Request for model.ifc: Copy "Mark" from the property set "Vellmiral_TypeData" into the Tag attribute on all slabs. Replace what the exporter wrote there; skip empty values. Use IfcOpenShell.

First a look at what the model holds.

```python
import ifcopenshell
import ifcopenshell.util.element

model = ifcopenshell.open("model.ifc")
print(model.schema)
slabs = model.by_type("IfcSlab")
print(len(slabs), "slabs")
for e in slabs[:8]:
    source = ifcopenshell.util.element.get_pset(e, "Vellmiral_TypeData", "Mark")
    target = e.Tag
    print(e.id(), repr(source), repr(target), sep=" | ")
```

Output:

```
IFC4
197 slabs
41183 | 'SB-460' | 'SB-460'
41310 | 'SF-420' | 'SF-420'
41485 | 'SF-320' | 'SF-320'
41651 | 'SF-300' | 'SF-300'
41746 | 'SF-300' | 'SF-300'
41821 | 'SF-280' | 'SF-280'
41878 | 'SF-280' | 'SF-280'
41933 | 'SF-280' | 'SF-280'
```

```python
import ifcopenshell
import ifcopenshell.util.element

model = ifcopenshell.open("model.ifc")

count = 0
for e in model.by_type("IfcSlab"):
    value = ifcopenshell.util.element.get_pset(e, "Vellmiral_TypeData", "Mark")
    current = e.Tag
    if not value or not value.strip() or current == value:
        continue
    e.Tag = value
    count += 1

print(count, "slabs updated")

model.write("model_v2.ifc")
```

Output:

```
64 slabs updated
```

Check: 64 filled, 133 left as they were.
